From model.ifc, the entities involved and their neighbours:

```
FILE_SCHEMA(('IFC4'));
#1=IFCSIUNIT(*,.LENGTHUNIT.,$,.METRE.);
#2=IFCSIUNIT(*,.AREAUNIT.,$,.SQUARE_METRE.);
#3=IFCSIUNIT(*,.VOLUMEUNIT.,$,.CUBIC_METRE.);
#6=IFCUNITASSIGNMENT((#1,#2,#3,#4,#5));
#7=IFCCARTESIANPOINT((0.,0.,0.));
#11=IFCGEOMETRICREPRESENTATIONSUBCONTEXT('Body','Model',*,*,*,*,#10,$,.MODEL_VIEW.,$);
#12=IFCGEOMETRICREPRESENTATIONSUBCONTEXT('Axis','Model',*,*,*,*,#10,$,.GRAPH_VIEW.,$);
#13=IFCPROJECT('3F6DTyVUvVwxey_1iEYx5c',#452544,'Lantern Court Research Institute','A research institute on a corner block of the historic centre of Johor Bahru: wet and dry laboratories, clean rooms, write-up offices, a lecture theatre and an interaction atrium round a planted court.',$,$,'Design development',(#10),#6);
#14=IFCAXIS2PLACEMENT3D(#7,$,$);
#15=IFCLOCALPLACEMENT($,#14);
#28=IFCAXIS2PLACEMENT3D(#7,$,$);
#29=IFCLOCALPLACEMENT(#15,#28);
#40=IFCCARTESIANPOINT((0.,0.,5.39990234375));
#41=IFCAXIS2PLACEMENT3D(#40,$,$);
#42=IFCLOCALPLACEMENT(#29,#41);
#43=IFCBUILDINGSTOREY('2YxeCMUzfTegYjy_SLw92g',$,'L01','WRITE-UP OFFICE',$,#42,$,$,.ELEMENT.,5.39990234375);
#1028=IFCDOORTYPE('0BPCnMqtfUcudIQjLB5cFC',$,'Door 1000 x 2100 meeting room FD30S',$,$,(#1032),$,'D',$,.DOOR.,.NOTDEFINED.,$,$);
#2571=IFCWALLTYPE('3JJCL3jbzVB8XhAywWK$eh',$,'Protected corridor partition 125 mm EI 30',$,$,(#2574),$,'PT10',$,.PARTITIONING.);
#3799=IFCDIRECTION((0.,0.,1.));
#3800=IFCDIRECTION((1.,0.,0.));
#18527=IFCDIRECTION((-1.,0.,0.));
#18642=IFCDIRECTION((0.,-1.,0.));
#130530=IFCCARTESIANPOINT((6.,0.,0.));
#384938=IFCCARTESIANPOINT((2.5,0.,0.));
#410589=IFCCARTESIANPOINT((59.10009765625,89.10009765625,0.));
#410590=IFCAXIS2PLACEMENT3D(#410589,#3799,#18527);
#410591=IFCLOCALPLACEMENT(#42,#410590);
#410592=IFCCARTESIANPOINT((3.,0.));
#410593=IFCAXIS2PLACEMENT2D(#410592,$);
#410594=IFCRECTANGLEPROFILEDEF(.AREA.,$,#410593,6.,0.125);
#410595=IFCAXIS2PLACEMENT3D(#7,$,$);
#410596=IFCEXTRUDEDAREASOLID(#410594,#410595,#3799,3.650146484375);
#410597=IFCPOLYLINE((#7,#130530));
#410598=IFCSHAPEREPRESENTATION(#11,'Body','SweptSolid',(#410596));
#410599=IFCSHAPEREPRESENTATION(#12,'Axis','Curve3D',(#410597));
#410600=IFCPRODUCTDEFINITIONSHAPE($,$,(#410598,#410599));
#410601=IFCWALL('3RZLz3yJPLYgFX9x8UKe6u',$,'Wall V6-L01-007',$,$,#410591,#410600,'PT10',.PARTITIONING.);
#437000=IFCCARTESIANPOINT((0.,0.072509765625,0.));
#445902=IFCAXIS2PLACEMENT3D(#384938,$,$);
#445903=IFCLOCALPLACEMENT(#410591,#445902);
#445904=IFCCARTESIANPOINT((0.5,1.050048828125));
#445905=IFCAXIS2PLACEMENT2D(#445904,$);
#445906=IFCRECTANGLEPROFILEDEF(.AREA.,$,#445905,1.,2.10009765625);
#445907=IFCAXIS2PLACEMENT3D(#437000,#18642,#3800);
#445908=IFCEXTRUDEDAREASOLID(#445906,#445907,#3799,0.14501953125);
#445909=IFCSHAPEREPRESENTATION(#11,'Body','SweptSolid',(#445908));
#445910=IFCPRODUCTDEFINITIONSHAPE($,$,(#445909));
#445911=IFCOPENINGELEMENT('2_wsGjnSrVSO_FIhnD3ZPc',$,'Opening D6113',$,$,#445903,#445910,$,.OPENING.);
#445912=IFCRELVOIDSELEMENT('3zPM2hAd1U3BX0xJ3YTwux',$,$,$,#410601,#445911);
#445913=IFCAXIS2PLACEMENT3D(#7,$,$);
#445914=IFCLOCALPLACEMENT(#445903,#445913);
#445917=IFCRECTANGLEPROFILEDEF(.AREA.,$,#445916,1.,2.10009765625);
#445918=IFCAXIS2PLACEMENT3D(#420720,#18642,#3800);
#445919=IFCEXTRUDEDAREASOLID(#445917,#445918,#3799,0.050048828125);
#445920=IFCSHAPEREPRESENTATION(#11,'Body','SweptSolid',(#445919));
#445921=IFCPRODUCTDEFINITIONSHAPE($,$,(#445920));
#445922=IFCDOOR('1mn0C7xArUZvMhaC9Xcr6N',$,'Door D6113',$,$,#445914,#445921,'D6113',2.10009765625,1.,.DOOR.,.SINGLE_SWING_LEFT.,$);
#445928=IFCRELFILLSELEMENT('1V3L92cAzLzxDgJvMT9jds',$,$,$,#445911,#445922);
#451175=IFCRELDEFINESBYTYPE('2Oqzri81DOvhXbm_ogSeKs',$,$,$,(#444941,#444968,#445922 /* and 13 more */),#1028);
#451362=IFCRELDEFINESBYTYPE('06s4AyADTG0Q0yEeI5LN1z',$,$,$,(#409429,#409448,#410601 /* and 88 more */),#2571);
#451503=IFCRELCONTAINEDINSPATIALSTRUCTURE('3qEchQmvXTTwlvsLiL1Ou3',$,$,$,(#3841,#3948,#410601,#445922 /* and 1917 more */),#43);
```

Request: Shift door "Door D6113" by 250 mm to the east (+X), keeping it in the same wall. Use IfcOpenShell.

```python
import ifcopenshell
import ifcopenshell.api.geometry
import ifcopenshell.util.placement
import ifcopenshell.util.unit

model = ifcopenshell.open("model.ifc")
unit_scale = ifcopenshell.util.unit.calculate_unit_scale(model)

door = model.by_id(445922)
opening = door.FillsVoids[0].RelatingOpeningElement
wall = opening.VoidsElements[0].RelatingBuildingElement

wall_matrix = ifcopenshell.util.placement.get_local_placement(wall.ObjectPlacement)
shift = wall_matrix[:3, 0] * -0.25 / unit_scale
before = ifcopenshell.util.placement.get_local_placement(door.ObjectPlacement)[:3, 3].copy()

# The door is placed relative to its opening, so it follows when the opening moves.
matrix = ifcopenshell.util.placement.get_local_placement(opening.ObjectPlacement)
matrix[:3, 3] += shift
ifcopenshell.api.geometry.edit_object_placement(
    model, product=opening, matrix=matrix, is_si=False, should_transform_children=True
)

after = ifcopenshell.util.placement.get_local_placement(door.ObjectPlacement)[:3, 3]
print("door moved by", (after - before).round(3) + 0.0)

model.write("model_edited.ifc")
```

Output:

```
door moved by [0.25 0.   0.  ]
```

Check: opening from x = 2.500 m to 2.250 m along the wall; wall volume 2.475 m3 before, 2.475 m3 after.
